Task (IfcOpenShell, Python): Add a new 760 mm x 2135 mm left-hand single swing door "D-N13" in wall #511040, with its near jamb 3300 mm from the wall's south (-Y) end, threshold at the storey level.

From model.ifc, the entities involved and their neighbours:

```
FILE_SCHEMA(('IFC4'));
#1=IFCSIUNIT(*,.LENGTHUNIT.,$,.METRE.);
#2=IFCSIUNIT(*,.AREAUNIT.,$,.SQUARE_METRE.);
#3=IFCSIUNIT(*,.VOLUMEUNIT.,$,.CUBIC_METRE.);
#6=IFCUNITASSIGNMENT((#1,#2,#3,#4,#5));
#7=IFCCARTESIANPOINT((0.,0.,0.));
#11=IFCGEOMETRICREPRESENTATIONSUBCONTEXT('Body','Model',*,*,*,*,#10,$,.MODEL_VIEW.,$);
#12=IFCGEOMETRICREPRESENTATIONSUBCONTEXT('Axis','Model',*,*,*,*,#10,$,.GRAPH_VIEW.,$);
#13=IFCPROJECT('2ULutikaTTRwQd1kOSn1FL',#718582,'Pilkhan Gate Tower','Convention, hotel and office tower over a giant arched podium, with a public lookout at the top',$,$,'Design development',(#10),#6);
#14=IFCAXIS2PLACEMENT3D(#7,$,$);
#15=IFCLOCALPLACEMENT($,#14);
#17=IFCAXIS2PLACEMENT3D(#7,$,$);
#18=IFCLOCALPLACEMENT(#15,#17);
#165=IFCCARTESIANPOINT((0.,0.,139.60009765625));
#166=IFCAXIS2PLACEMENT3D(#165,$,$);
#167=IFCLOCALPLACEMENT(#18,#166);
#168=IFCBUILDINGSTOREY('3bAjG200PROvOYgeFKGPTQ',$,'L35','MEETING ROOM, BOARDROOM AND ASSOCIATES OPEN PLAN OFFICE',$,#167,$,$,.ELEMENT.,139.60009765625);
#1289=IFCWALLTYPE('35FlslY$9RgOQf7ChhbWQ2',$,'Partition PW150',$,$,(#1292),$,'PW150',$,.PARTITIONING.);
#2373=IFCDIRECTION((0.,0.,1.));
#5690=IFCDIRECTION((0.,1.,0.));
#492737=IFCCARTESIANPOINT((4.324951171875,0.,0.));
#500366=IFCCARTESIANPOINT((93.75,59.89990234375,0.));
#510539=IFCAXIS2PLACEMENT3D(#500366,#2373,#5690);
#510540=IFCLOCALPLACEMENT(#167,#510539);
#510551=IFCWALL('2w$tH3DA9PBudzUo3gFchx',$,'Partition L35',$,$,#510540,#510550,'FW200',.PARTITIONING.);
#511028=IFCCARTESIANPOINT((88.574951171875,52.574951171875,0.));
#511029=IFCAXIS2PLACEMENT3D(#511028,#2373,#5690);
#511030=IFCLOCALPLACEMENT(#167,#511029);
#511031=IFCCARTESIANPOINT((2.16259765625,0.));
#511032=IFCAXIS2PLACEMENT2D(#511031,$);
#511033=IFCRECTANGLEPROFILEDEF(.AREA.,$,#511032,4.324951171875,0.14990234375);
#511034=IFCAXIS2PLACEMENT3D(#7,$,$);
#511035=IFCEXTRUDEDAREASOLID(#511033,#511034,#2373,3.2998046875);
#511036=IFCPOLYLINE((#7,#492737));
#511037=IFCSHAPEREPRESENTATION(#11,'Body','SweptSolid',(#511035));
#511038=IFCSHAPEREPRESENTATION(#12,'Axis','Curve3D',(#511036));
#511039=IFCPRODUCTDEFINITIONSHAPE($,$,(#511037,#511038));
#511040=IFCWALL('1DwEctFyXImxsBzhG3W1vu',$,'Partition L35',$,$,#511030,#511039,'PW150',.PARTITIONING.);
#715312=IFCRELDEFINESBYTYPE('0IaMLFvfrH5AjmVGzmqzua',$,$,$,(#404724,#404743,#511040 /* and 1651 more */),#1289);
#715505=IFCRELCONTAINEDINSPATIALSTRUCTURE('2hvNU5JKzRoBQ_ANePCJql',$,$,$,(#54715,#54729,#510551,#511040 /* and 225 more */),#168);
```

```python
import numpy as np
import ifcopenshell
import ifcopenshell.api.feature
import ifcopenshell.api.geometry
import ifcopenshell.api.root
import ifcopenshell.api.spatial
import ifcopenshell.geom
import ifcopenshell.util.element
import ifcopenshell.util.placement
import ifcopenshell.util.representation
import ifcopenshell.util.shape
import ifcopenshell.util.unit

model = ifcopenshell.open("model.ifc")
unit_scale = ifcopenshell.util.unit.calculate_unit_scale(model)
settings = ifcopenshell.geom.settings()


def volume(element):
    """Net volume in cubic metres, openings subtracted."""
    shape = ifcopenshell.geom.create_shape(settings, element)
    return ifcopenshell.util.shape.get_volume(shape.geometry)


wall = model.by_id(511040)
storey = ifcopenshell.util.element.get_container(wall, ifc_class="IfcBuildingStorey")
context = ifcopenshell.util.representation.get_context(model, "Model", "Body", "MODEL_VIEW")
before = volume(wall)

width, height, from_end, sill = 0.76, 2.135, 3.3, 0.0  # metres

# The wall runs along its own X axis, and the end named is its -X end.
wall_shape = ifcopenshell.geom.create_shape(settings, wall)
x, y, z = ifcopenshell.util.shape.get_vertices(wall_shape.geometry).T
start = x.min() + from_end
face, thickness = float(y.min()), float(y.max() - y.min())
wall_matrix = ifcopenshell.util.placement.get_local_placement(wall.ObjectPlacement)
level = ifcopenshell.util.placement.get_local_placement(storey.ObjectPlacement)[2, 3]


def in_wall(x, y):
    """Placement at x, y metres in the wall's axes, at sill height."""
    matrix = wall_matrix.copy()
    matrix[:, 3] = wall_matrix @ np.array([x / unit_scale, y / unit_scale, 0.0, 1.0])
    matrix[2, 3] = level + sill / unit_scale
    return matrix


# Opening: a box that overshoots both wall faces by 50 mm.
opening = ifcopenshell.api.root.create_entity(model, ifc_class="IfcOpeningElement", predefined_type="OPENING")
box = ifcopenshell.api.geometry.add_wall_representation(
    model, context=context, length=width, height=height, thickness=thickness + 0.1
)
ifcopenshell.api.geometry.assign_representation(model, product=opening, representation=box)
ifcopenshell.api.geometry.edit_object_placement(model, product=opening, matrix=in_wall(start, face - 0.05), is_si=False)
ifcopenshell.api.feature.add_feature(model, feature=opening, element=wall)

door = ifcopenshell.api.root.create_entity(model, ifc_class="IfcDoor", name="D-N13", predefined_type="DOOR")
door.OverallWidth, door.OverallHeight = width / unit_scale, height / unit_scale
door.OperationType = "SINGLE_SWING_LEFT"
body = ifcopenshell.api.geometry.add_door_representation(
    model,
    context=context,
    overall_width=door.OverallWidth,
    overall_height=door.OverallHeight,
    operation_type="SINGLE_SWING_LEFT",
    lining_properties={"LiningDepth": thickness / unit_scale, "ThresholdDepth": thickness / unit_scale},
)
ifcopenshell.api.geometry.assign_representation(model, product=door, representation=body)
ifcopenshell.api.spatial.assign_container(model, products=[door], relating_structure=storey)
ifcopenshell.api.feature.add_filling(model, opening=opening, element=door)

# The lining spans the wall, so the door starts at the wall face.
ifcopenshell.api.geometry.edit_object_placement(model, product=door, matrix=in_wall(start, face), is_si=False)

after = volume(wall)

print(f"wall volume {before:.3f} -> {after:.3f} m3")

model.write("model_v2.ifc")
```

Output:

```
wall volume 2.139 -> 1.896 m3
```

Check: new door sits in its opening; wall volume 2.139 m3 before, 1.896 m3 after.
